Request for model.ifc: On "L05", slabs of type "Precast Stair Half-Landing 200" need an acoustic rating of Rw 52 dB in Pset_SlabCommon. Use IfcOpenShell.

First a look at what the model holds.

```python
import ifcopenshell
import ifcopenshell.util.element

model = ifcopenshell.open("model.ifc")
print(model.schema)
storey = next(s for s in model.by_type("IfcBuildingStorey") if s.Name == "L05")
slabs = [e for e in ifcopenshell.util.element.get_decomposition(storey) if e.is_a("IfcSlab")]
seen = {}
for e in slabs:
    element_type = ifcopenshell.util.element.get_type(e)
    key = (element_type.Name if element_type != e and element_type else None, ifcopenshell.util.element.get_pset(e, "Pset_SlabCommon", "AcousticRating"))
    seen[key] = seen.get(key, 0) + 1
for (name, value), count in sorted(seen.items(), key=str):
    print(count, "x", name, "|", value)
```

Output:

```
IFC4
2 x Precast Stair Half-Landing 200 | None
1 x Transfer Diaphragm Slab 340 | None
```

```python
import ifcopenshell
import ifcopenshell.api.pset
import ifcopenshell.util.element

model = ifcopenshell.open("model.ifc")

storey = next(s for s in model.by_type("IfcBuildingStorey") if s.Name == "L05")
slabs = [e for e in ifcopenshell.util.element.get_decomposition(storey) if e.is_a("IfcSlab")]

count = 0
for e in slabs:
    element_type = ifcopenshell.util.element.get_type(e)
    if element_type in (None, e) or element_type.Name != "Precast Stair Half-Landing 200":
        continue
    found = ifcopenshell.util.element.get_pset(e, "Pset_SlabCommon", should_inherit=False)
    if found:
        pset = model.by_id(found["id"])
        if len(ifcopenshell.util.element.get_elements_by_pset(pset)) > 1:
            pset = ifcopenshell.api.pset.unshare_pset(model, products=[e], pset=pset)[0]
    else:
        pset = ifcopenshell.api.pset.add_pset(model, product=e, name="Pset_SlabCommon")
    ifcopenshell.api.pset.edit_pset(model, pset=pset, properties={"AcousticRating": "Rw 52 dB"})
    count += 1

print(count, "slabs updated")

model.write("model-out.ifc")
```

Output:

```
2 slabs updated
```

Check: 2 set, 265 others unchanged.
